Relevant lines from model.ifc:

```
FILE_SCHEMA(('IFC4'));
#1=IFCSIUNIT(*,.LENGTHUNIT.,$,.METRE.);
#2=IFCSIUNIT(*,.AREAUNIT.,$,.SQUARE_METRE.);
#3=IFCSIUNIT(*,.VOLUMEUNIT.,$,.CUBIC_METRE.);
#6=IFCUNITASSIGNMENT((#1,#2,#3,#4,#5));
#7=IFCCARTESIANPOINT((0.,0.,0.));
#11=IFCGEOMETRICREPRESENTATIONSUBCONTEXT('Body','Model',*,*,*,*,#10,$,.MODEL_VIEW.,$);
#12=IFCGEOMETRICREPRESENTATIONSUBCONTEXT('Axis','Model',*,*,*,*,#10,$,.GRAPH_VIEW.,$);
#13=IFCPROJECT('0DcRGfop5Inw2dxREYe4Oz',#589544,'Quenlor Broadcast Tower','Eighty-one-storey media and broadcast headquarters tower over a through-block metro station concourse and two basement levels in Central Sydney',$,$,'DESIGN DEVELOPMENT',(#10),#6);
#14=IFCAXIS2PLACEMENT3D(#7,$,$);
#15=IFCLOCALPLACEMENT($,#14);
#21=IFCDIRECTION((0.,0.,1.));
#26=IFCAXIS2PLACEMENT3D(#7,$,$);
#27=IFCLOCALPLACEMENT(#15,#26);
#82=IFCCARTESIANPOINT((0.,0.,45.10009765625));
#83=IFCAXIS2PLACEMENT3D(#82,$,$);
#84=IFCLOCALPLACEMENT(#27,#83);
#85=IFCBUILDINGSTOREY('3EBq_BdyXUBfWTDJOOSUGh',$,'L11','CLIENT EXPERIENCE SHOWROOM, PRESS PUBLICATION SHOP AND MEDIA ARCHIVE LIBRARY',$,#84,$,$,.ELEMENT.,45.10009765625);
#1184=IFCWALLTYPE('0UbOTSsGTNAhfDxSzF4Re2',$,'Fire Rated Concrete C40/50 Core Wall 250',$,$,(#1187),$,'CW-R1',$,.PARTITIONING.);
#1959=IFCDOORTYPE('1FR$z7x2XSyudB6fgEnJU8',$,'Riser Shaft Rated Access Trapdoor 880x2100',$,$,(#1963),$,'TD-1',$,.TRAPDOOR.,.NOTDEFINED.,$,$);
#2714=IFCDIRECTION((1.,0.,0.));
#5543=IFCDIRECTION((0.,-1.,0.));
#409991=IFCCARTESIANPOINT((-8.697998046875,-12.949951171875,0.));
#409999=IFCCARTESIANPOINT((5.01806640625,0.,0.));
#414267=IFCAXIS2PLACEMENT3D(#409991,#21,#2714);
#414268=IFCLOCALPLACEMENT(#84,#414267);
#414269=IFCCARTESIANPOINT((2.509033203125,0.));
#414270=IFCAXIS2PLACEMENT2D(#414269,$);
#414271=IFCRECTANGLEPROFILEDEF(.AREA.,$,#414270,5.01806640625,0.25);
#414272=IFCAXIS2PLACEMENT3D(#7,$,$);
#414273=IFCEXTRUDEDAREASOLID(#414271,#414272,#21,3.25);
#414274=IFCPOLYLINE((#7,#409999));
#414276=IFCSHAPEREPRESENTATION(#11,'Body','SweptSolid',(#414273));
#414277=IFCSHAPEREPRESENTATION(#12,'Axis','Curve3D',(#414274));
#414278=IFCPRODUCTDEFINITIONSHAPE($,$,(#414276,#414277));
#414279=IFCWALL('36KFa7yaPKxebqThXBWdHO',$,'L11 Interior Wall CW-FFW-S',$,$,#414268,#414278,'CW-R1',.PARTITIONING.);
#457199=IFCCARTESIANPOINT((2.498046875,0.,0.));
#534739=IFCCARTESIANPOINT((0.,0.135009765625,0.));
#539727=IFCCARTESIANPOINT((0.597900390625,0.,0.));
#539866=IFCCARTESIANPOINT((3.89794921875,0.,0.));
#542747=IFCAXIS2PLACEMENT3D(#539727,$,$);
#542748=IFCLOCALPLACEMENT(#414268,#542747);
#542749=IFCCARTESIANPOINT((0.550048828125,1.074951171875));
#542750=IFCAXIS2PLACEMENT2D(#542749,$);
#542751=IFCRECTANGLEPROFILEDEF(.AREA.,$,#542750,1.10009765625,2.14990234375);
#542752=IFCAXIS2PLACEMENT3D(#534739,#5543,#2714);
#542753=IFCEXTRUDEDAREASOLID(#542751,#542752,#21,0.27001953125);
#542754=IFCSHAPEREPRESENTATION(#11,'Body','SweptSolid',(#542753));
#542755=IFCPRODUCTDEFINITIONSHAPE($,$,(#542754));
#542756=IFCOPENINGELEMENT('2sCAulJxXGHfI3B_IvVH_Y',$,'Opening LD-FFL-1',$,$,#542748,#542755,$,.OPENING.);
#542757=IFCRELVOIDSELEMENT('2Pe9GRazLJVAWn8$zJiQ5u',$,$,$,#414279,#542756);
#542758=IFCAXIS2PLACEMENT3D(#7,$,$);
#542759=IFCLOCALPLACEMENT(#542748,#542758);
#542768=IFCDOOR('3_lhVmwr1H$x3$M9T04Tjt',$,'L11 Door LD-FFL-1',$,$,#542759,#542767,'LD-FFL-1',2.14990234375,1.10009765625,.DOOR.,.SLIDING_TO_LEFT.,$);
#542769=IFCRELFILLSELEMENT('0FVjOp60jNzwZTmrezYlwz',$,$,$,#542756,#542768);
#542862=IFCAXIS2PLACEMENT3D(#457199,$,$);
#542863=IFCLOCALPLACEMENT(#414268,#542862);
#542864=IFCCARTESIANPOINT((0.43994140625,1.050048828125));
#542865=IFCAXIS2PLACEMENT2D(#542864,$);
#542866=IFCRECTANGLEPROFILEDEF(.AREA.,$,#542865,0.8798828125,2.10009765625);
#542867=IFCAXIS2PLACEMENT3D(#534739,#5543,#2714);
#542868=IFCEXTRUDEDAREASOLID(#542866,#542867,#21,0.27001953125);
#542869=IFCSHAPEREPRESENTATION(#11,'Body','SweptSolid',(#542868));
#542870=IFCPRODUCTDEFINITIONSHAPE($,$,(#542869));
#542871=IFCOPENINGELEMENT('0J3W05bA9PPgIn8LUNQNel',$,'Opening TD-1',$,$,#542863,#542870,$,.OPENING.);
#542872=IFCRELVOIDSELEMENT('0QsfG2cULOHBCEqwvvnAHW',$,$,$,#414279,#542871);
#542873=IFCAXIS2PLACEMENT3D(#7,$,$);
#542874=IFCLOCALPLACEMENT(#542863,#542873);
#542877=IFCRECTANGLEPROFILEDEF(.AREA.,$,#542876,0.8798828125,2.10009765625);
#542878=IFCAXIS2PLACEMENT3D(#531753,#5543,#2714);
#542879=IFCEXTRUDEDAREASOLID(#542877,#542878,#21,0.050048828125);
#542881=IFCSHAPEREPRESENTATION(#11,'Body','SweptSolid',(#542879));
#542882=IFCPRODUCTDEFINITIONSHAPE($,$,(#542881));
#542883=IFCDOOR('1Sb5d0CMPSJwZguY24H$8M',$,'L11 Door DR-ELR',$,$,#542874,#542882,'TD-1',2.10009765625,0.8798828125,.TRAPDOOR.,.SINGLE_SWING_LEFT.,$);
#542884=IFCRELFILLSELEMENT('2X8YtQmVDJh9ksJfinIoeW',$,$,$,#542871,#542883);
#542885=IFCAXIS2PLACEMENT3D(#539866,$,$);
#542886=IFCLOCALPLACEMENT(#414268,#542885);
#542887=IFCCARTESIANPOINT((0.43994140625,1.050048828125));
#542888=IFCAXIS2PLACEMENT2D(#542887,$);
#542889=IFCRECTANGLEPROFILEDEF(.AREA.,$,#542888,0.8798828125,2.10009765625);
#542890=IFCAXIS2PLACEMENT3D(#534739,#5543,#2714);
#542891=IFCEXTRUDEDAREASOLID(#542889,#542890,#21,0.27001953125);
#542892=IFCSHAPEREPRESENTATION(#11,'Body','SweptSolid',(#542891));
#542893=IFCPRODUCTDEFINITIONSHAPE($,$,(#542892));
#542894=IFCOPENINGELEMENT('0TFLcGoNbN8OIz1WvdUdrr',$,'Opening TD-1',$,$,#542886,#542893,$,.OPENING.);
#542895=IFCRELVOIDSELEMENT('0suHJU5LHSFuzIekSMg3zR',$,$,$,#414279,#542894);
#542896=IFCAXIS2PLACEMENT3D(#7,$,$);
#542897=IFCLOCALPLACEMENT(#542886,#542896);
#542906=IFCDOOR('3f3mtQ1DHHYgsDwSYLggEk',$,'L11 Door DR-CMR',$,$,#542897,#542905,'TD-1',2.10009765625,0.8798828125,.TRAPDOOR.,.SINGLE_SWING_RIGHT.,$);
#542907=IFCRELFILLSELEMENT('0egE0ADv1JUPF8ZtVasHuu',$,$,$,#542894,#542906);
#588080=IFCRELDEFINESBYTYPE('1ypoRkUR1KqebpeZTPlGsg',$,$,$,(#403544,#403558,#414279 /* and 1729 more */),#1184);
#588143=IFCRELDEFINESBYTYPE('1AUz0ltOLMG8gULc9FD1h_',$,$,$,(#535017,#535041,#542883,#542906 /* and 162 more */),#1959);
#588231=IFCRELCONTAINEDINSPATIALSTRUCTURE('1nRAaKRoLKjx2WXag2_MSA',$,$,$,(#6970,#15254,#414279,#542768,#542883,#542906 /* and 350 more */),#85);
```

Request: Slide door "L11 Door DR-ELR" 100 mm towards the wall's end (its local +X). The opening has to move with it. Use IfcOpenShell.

```python
import ifcopenshell
import ifcopenshell.api.geometry
import ifcopenshell.util.placement
import ifcopenshell.util.unit

model = ifcopenshell.open("model.ifc")
unit_scale = ifcopenshell.util.unit.calculate_unit_scale(model)

door = model.by_guid("1Sb5d0CMPSJwZguY24H$8M")
opening = door.FillsVoids[0].RelatingOpeningElement
wall = opening.VoidsElements[0].RelatingBuildingElement

wall_matrix = ifcopenshell.util.placement.get_local_placement(wall.ObjectPlacement)
shift = wall_matrix[:3, 0] * 0.1 / unit_scale
before = ifcopenshell.util.placement.get_local_placement(door.ObjectPlacement)[:3, 3].copy()

# The door is placed relative to its opening, so it follows when the opening moves.
matrix = ifcopenshell.util.placement.get_local_placement(opening.ObjectPlacement)
matrix[:3, 3] += shift
ifcopenshell.api.geometry.edit_object_placement(
    model, product=opening, matrix=matrix, is_si=False, should_transform_children=True
)

after = ifcopenshell.util.placement.get_local_placement(door.ObjectPlacement)[:3, 3]
print("door moved by", (after - before).round(3) + 0.0)

model.write("model-out.ifc")
```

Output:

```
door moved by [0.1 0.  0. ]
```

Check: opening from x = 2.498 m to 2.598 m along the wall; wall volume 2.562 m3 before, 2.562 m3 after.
